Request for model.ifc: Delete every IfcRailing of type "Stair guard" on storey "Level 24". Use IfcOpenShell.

First a look at what the model holds.

```python
import ifcopenshell
import ifcopenshell.util.element

model = ifcopenshell.open("model.ifc")
print(model.schema)
storey = next(s for s in model.by_type("IfcBuildingStorey") if s.Name == "Level 24")
railings = [e for e in ifcopenshell.util.element.get_decomposition(storey) if e.is_a("IfcRailing")]
seen = {}
for e in railings:
    element_type = ifcopenshell.util.element.get_type(e)
    name = element_type.Name if element_type not in (None, e) else None
    seen[name] = seen.get(name, 0) + 1
for name, count in sorted(seen.items(), key=str):
    print(count, "x", name)
```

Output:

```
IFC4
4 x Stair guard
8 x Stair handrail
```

```python
import ifcopenshell
import ifcopenshell.api.root
import ifcopenshell.util.element

model = ifcopenshell.open("model.ifc")

storey = next(s for s in model.by_type("IfcBuildingStorey") if s.Name == "Level 24")
railings = [e for e in ifcopenshell.util.element.get_decomposition(storey) if e.is_a("IfcRailing")]
targets = [e for e in railings if (t := ifcopenshell.util.element.get_type(e)) not in (None, e) and t.Name == "Stair guard"]

for e in targets:
    ifcopenshell.api.root.remove_product(model, product=e)
print(len(targets), "removed")

model.write("model-out.ifc")
```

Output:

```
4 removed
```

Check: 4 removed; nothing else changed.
